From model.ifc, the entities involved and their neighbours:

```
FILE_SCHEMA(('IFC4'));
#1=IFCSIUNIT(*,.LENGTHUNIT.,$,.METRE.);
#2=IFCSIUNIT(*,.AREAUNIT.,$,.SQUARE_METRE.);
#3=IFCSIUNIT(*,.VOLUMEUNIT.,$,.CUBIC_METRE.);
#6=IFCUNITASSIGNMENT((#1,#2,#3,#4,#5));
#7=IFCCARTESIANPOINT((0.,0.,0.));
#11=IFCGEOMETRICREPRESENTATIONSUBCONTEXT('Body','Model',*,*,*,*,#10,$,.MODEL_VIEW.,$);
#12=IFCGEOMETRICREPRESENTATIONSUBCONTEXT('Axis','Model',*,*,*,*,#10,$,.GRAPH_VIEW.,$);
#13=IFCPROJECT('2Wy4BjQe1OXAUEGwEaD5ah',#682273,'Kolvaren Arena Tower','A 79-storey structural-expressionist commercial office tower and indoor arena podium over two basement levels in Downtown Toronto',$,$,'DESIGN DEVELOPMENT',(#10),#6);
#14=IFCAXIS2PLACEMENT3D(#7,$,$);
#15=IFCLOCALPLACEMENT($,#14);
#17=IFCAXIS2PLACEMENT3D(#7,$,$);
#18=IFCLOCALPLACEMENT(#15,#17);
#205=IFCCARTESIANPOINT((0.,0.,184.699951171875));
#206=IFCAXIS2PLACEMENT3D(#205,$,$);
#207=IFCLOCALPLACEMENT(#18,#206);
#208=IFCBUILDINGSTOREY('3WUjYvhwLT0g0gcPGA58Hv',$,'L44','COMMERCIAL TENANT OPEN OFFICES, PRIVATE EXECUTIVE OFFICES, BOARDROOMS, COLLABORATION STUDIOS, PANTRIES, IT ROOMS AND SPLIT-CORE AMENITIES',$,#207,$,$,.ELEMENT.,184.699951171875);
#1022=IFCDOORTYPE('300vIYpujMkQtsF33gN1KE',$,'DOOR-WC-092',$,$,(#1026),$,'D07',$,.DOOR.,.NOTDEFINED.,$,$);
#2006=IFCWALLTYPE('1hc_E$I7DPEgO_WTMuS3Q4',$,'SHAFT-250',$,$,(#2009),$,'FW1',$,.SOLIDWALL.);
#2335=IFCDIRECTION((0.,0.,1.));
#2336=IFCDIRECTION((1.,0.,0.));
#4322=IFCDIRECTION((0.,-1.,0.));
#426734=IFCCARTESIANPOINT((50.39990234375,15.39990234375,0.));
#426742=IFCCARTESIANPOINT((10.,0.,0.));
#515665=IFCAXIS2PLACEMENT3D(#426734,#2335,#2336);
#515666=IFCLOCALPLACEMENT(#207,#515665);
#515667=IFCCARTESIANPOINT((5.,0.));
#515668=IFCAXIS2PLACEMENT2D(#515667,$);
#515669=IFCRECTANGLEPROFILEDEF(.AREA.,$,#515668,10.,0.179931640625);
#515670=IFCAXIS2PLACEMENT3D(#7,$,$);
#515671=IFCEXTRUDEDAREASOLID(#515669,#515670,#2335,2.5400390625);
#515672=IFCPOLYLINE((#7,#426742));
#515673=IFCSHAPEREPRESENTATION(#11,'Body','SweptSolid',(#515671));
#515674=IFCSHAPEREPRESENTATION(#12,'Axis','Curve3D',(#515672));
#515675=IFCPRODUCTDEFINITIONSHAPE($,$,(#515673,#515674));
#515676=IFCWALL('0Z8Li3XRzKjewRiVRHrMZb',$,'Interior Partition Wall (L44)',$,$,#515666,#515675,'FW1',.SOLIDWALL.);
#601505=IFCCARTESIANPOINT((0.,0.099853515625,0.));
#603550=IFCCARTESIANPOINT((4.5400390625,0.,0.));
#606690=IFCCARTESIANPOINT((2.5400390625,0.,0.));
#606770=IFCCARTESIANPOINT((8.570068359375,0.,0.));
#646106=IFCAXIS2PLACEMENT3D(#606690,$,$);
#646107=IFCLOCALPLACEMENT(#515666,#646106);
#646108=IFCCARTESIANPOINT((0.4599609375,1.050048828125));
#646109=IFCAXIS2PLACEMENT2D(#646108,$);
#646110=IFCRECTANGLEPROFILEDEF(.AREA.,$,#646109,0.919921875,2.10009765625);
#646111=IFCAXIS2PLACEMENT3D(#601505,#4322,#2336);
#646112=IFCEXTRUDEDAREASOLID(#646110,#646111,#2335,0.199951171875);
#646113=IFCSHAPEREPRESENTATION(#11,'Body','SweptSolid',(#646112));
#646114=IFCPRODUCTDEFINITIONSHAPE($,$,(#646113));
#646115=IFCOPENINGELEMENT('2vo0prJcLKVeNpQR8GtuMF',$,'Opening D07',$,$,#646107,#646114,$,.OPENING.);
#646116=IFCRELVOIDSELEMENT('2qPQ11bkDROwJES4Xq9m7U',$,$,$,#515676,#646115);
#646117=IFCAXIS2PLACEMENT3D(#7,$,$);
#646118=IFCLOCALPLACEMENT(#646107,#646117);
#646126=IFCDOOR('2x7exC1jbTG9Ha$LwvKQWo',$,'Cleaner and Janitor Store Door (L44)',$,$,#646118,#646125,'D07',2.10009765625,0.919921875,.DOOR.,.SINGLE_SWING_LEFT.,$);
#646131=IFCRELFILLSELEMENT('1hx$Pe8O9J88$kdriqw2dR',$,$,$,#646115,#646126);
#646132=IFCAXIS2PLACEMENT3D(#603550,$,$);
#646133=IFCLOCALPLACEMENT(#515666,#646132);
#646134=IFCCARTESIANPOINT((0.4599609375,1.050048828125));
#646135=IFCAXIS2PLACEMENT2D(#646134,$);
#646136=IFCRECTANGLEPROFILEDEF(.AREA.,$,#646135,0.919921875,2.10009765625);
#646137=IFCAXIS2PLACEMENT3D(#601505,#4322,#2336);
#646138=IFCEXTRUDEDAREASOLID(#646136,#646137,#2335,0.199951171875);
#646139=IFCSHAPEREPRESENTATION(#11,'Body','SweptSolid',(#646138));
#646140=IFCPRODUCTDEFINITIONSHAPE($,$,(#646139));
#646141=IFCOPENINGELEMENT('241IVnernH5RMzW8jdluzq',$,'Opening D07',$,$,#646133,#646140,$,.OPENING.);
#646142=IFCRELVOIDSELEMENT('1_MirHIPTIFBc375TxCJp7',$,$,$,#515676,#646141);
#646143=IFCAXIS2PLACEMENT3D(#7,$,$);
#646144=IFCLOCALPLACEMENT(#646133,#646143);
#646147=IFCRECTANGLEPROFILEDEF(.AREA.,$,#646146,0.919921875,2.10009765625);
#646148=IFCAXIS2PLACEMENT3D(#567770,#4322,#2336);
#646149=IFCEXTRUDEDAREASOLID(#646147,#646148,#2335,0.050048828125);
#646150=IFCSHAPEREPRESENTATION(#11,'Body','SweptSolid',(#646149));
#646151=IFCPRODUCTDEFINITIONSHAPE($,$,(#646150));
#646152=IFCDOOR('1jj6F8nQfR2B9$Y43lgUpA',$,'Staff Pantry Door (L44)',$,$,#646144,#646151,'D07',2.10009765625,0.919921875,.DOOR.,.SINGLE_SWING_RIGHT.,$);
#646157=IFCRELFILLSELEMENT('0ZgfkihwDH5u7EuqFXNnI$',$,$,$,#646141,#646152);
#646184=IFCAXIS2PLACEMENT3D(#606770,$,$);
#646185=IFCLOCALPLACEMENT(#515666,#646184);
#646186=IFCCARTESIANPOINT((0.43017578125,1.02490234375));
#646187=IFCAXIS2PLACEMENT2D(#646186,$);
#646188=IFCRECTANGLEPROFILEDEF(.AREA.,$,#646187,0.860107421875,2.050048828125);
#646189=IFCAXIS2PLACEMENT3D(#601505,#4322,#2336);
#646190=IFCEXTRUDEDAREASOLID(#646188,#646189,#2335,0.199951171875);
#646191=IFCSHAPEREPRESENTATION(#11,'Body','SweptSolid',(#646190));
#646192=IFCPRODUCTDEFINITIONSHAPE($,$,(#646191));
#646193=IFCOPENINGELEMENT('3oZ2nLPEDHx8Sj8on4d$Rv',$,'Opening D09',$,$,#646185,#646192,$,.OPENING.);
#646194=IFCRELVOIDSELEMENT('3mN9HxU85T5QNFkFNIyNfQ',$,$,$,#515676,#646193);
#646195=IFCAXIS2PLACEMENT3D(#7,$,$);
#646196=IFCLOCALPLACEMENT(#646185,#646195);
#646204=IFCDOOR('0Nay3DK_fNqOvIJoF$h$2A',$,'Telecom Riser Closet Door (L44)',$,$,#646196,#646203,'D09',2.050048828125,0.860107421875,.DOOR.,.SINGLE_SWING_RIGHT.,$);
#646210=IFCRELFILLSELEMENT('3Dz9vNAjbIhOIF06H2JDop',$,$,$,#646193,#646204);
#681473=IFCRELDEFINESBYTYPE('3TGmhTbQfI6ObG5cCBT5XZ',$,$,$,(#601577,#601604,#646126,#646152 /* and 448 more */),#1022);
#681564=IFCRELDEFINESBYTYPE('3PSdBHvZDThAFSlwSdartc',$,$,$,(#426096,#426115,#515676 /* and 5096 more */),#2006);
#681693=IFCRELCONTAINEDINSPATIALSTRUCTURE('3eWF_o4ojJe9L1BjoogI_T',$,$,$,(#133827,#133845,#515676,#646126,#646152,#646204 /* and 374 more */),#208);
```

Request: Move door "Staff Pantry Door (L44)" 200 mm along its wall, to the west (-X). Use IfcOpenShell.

```python
import ifcopenshell
import ifcopenshell.api.geometry
import ifcopenshell.util.placement
import ifcopenshell.util.unit

model = ifcopenshell.open("model.ifc")
unit_scale = ifcopenshell.util.unit.calculate_unit_scale(model)

door = model.by_guid("1jj6F8nQfR2B9$Y43lgUpA")
opening = door.FillsVoids[0].RelatingOpeningElement
wall = opening.VoidsElements[0].RelatingBuildingElement

wall_matrix = ifcopenshell.util.placement.get_local_placement(wall.ObjectPlacement)
shift = wall_matrix[:3, 0] * -0.2 / unit_scale
before = ifcopenshell.util.placement.get_local_placement(door.ObjectPlacement)[:3, 3].copy()

# The door is placed relative to its opening, so it follows when the opening moves.
matrix = ifcopenshell.util.placement.get_local_placement(opening.ObjectPlacement)
matrix[:3, 3] += shift
ifcopenshell.api.geometry.edit_object_placement(
    model, product=opening, matrix=matrix, is_si=False, should_transform_children=True
)

after = ifcopenshell.util.placement.get_local_placement(door.ObjectPlacement)[:3, 3]
print("door moved by", (after - before).round(3) + 0.0)

model.write("model_v2.ifc")
```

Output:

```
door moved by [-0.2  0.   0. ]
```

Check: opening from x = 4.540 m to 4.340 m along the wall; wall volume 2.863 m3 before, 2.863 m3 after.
